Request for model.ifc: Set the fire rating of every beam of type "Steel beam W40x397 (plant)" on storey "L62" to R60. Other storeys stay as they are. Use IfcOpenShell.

First a look at what the model holds.

```python
import ifcopenshell
import ifcopenshell.util.element

model = ifcopenshell.open("model.ifc")
print(model.schema)
storey = next(s for s in model.by_type("IfcBuildingStorey") if s.Name == "L62")
beams = [e for e in ifcopenshell.util.element.get_decomposition(storey) if e.is_a("IfcBeam")]
seen = {}
for e in beams:
    element_type = ifcopenshell.util.element.get_type(e)
    key = (element_type.Name if element_type != e and element_type else None, ifcopenshell.util.element.get_pset(e, "Pset_BeamCommon", "FireRating"))
    seen[key] = seen.get(key, 0) + 1
for (name, value), count in sorted(seen.items(), key=str):
    print(count, "x", name, "|", value)
```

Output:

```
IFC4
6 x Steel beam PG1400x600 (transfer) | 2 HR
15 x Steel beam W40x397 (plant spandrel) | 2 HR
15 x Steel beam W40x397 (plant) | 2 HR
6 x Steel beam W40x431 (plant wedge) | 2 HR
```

```python
import ifcopenshell
import ifcopenshell.api.pset
import ifcopenshell.util.element

model = ifcopenshell.open("model.ifc")

storey = next(s for s in model.by_type("IfcBuildingStorey") if s.Name == "L62")
beams = [e for e in ifcopenshell.util.element.get_decomposition(storey) if e.is_a("IfcBeam")]

count = 0
for e in beams:
    element_type = ifcopenshell.util.element.get_type(e)
    if element_type in (None, e) or element_type.Name != "Steel beam W40x397 (plant)":
        continue
    found = ifcopenshell.util.element.get_pset(e, "Pset_BeamCommon", should_inherit=False)
    if found:
        pset = model.by_id(found["id"])
        if len(ifcopenshell.util.element.get_elements_by_pset(pset)) > 1:
            pset = ifcopenshell.api.pset.unshare_pset(model, products=[e], pset=pset)[0]
    else:
        pset = ifcopenshell.api.pset.add_pset(model, product=e, name="Pset_BeamCommon")
    ifcopenshell.api.pset.edit_pset(model, pset=pset, properties={"FireRating": "R60"})
    count += 1

print(count, "beams updated")

model.write("model_updated.ifc")
```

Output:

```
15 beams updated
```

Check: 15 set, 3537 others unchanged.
